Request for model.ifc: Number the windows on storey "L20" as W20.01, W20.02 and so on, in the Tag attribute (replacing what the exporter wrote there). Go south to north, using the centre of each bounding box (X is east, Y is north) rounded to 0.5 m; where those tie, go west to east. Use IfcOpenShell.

First a look at what the model holds.

```python
import ifcopenshell
import ifcopenshell.util.element
import ifcopenshell.util.placement

model = ifcopenshell.open("model.ifc")
print(model.schema)
storey = next(s for s in model.by_type("IfcBuildingStorey") if s.Name == "L20")
windows = [e for e in ifcopenshell.util.element.get_decomposition(storey) if e.is_a("IfcWindow")]
for e in sorted(windows, key=lambda e: e.id()):
    origin = ifcopenshell.util.placement.get_local_placement(e.ObjectPlacement)[:3, 3]
    print(e.id(), e.Tag, e.Name, origin.round(2) + 0.0, sep=" | ")
```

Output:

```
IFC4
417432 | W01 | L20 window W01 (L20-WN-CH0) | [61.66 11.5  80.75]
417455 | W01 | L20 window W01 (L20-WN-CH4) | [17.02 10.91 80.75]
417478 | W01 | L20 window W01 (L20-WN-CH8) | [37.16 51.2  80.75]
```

```python
import ifcopenshell
import ifcopenshell.geom
import ifcopenshell.util.element
import ifcopenshell.util.shape

model = ifcopenshell.open("model.ifc")
settings = ifcopenshell.geom.settings()
settings.set("use-world-coords", True)


def centre(element):
    shape = ifcopenshell.geom.create_shape(settings, element)
    return ifcopenshell.util.shape.get_bbox_centroid(shape.geometry)


storey = next(s for s in model.by_type("IfcBuildingStorey") if s.Name == "L20")
windows = [e for e in ifcopenshell.util.element.get_decomposition(storey) if e.is_a("IfcWindow")]

# Insertion points can sit at a corner or the storey origin, so sort by the geometry (in metres).
centres = {e: centre(e) for e in windows}
windows.sort(key=lambda e: (round(centres[e][1] / 0.5), centres[e][0]))

for i, e in enumerate(windows, start=1):
    number = f"W20.{i:02d}"
    e.Tag = number
    print(e.id(), number)

model.write("model_v2.ifc")
```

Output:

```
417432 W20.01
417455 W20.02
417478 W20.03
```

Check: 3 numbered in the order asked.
